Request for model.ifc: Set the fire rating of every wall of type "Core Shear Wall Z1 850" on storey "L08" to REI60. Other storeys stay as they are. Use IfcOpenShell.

First a look at what the model holds.

```python
import ifcopenshell
import ifcopenshell.util.element

model = ifcopenshell.open("model.ifc")
print(model.schema)
storey = next(s for s in model.by_type("IfcBuildingStorey") if s.Name == "L08")
walls = [e for e in ifcopenshell.util.element.get_decomposition(storey) if e.is_a("IfcWall")]
seen = {}
for e in walls:
    element_type = ifcopenshell.util.element.get_type(e)
    key = (element_type.Name if element_type != e and element_type else None, ifcopenshell.util.element.get_pset(e, "Pset_WallCommon", "FireRating"))
    seen[key] = seen.get(key, 0) + 1
for (name, value), count in sorted(seen.items(), key=str):
    print(count, "x", name, "|", value)
```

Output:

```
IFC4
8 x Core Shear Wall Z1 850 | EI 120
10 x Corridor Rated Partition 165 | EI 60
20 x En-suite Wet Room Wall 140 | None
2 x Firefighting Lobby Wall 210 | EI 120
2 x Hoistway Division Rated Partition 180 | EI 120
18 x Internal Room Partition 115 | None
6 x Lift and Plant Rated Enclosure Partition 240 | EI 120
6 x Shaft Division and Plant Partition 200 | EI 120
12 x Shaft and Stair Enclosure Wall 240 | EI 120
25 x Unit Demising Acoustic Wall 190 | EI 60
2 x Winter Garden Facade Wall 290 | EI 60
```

```python
import ifcopenshell
import ifcopenshell.api.pset
import ifcopenshell.util.element

model = ifcopenshell.open("model.ifc")

storey = next(s for s in model.by_type("IfcBuildingStorey") if s.Name == "L08")
walls = [e for e in ifcopenshell.util.element.get_decomposition(storey) if e.is_a("IfcWall")]

count = 0
for e in walls:
    element_type = ifcopenshell.util.element.get_type(e)
    if element_type in (None, e) or element_type.Name != "Core Shear Wall Z1 850":
        continue
    found = ifcopenshell.util.element.get_pset(e, "Pset_WallCommon", should_inherit=False)
    if found:
        pset = model.by_id(found["id"])
        if len(ifcopenshell.util.element.get_elements_by_pset(pset)) > 1:
            pset = ifcopenshell.api.pset.unshare_pset(model, products=[e], pset=pset)[0]
    else:
        pset = ifcopenshell.api.pset.add_pset(model, product=e, name="Pset_WallCommon")
    ifcopenshell.api.pset.edit_pset(model, pset=pset, properties={"FireRating": "REI60"})
    count += 1

print(count, "walls updated")

model.write("model_v2.ifc")
```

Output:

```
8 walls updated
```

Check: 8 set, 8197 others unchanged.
